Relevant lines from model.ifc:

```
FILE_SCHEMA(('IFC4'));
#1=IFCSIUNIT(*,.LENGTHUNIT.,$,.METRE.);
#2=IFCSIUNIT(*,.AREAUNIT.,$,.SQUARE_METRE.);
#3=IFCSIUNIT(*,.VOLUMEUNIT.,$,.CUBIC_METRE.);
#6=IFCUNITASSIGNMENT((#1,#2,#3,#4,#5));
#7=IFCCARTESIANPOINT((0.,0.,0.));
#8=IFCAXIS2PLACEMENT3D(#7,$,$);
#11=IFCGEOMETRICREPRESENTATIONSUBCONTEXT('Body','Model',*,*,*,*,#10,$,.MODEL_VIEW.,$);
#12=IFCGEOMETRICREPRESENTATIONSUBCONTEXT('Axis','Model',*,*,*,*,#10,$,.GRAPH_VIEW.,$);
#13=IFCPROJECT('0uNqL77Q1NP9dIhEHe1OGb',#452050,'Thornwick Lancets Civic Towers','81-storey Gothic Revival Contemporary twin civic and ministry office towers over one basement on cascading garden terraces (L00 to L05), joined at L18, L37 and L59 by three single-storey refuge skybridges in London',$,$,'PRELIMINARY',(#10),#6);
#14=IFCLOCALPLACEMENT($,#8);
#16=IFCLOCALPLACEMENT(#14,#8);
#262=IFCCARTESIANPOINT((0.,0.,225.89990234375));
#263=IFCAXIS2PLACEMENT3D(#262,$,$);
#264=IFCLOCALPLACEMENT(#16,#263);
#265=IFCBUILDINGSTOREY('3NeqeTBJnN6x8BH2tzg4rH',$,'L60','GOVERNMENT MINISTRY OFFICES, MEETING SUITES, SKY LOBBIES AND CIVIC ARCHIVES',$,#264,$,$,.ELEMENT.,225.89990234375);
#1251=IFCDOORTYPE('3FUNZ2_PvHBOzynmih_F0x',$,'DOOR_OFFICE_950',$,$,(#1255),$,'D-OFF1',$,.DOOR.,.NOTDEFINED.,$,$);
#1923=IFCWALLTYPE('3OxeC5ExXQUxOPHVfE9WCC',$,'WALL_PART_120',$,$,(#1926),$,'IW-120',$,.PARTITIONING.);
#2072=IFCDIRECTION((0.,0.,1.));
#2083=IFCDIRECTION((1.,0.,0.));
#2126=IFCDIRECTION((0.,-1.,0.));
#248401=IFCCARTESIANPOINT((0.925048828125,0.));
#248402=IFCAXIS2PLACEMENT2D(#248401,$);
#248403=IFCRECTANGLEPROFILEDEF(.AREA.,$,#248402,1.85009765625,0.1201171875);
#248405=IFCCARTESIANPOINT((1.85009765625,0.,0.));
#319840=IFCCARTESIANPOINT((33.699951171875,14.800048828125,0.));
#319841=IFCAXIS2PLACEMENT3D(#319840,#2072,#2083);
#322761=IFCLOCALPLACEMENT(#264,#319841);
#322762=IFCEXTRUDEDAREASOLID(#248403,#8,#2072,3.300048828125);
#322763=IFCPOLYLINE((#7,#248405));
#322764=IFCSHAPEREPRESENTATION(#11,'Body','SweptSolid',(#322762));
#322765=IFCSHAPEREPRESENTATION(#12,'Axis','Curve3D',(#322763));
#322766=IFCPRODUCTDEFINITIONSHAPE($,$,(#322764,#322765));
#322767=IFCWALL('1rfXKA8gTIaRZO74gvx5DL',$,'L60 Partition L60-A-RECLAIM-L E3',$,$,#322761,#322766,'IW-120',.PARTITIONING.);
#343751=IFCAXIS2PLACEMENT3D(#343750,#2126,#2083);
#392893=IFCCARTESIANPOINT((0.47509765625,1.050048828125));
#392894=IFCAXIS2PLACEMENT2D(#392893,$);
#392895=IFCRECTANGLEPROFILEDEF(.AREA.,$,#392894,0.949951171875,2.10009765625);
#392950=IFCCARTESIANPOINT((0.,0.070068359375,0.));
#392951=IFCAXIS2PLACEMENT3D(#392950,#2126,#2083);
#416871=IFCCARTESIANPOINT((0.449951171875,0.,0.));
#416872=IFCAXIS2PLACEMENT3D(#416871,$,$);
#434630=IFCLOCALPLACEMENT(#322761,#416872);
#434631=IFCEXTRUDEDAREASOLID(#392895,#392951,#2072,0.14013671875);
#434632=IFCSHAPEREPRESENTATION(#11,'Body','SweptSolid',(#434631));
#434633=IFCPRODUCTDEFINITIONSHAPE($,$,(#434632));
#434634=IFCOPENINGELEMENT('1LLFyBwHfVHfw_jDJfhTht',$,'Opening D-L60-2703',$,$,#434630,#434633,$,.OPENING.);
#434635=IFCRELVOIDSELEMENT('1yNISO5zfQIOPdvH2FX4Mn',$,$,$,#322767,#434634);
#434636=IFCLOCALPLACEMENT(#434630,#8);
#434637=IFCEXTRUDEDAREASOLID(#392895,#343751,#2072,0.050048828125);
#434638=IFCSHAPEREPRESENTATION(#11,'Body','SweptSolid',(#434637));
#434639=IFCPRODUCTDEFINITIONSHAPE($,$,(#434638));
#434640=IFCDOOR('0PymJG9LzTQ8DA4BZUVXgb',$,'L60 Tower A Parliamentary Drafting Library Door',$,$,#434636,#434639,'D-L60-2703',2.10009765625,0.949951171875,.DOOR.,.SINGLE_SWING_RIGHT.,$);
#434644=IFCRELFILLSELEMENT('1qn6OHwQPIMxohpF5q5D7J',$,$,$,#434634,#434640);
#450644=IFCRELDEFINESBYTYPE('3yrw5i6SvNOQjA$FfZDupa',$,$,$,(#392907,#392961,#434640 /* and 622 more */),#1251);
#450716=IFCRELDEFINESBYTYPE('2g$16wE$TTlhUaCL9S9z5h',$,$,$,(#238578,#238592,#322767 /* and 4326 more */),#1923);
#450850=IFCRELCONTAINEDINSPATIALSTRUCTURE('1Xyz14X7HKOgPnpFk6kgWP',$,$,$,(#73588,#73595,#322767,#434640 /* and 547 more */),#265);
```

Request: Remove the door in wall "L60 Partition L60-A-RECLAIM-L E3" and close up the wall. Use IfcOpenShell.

```python
import ifcopenshell
import ifcopenshell.api.feature
import ifcopenshell.api.root
import ifcopenshell.geom
import ifcopenshell.util.shape

model = ifcopenshell.open("model.ifc")
settings = ifcopenshell.geom.settings()


def volume(element):
    """Net volume in cubic metres, openings subtracted."""
    shape = ifcopenshell.geom.create_shape(settings, element)
    return ifcopenshell.util.shape.get_volume(shape.geometry)


door = model.by_guid("0PymJG9LzTQ8DA4BZUVXgb")
opening = door.FillsVoids[0].RelatingOpeningElement
wall = opening.VoidsElements[0].RelatingBuildingElement
before = volume(wall)

ifcopenshell.api.root.remove_product(model, product=door)
ifcopenshell.api.feature.remove_feature(model, feature=opening)

after = volume(wall)

print(f"wall volume {before:.3f} -> {after:.3f} m3")

model.write("model-out.ifc")
```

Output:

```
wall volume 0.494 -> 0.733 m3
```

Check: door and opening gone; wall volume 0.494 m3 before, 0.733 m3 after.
